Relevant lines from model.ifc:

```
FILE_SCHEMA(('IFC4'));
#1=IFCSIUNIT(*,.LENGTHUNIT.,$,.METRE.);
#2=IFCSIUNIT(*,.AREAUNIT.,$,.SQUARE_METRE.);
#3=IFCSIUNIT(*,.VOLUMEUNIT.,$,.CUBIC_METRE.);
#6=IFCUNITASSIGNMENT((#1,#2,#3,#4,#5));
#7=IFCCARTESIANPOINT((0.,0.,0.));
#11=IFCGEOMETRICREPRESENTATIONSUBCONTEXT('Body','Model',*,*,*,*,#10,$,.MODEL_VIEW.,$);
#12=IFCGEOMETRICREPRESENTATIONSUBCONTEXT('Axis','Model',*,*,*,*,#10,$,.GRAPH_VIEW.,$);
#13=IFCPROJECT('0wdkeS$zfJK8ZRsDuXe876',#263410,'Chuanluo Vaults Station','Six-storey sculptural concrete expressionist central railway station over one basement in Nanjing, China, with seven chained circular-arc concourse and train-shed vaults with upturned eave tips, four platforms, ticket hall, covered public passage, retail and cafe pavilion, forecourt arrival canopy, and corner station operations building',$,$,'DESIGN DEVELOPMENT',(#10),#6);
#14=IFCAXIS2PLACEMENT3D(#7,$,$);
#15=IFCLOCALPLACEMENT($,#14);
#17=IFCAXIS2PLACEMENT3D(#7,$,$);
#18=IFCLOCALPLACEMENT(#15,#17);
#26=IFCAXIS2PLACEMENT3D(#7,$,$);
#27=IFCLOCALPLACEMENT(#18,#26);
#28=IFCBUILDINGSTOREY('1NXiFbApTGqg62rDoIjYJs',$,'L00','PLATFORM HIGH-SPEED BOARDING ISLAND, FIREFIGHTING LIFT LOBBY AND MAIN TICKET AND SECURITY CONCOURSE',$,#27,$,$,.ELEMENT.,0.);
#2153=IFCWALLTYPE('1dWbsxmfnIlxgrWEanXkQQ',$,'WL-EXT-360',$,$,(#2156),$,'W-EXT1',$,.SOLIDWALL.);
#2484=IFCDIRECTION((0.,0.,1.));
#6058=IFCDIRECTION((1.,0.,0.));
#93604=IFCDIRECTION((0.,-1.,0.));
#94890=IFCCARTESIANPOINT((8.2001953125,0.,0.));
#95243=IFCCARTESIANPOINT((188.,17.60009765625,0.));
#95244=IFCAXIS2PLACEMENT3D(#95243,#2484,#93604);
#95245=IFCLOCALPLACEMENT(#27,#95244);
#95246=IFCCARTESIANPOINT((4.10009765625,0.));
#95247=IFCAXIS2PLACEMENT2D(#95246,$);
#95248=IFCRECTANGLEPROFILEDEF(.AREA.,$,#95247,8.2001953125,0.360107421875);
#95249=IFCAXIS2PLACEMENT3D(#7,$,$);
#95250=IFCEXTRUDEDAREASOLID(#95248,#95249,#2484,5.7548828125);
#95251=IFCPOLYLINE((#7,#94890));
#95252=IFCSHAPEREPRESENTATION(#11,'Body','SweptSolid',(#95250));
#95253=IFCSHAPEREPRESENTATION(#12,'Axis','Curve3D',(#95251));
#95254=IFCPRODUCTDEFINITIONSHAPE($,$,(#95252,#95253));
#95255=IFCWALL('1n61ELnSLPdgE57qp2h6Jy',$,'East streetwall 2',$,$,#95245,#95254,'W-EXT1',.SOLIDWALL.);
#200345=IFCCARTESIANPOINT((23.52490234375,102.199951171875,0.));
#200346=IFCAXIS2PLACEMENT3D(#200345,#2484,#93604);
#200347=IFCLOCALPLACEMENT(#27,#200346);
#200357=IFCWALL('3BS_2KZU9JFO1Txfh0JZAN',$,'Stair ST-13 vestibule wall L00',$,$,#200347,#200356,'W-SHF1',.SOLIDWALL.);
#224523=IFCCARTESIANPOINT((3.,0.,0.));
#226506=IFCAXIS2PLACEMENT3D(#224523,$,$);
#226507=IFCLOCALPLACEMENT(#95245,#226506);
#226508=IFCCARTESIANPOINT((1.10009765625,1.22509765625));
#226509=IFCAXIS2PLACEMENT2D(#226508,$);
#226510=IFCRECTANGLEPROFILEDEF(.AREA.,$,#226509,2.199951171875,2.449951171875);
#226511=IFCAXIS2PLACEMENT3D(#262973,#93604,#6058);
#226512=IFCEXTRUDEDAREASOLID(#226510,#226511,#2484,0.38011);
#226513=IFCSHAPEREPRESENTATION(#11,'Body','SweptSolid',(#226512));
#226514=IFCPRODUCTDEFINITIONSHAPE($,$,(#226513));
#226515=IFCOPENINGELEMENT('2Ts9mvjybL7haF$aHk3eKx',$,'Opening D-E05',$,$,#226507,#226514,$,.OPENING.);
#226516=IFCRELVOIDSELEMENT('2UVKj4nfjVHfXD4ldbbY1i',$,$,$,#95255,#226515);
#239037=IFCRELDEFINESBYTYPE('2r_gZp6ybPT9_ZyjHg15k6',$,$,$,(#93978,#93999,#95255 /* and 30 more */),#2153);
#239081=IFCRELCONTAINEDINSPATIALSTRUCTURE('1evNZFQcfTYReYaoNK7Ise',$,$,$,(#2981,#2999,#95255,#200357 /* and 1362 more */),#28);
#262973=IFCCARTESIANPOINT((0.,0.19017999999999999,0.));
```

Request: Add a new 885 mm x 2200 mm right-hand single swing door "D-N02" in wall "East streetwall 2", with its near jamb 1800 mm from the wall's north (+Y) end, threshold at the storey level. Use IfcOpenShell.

```python
import numpy as np
import ifcopenshell
import ifcopenshell.api.feature
import ifcopenshell.api.geometry
import ifcopenshell.api.root
import ifcopenshell.api.spatial
import ifcopenshell.geom
import ifcopenshell.util.element
import ifcopenshell.util.placement
import ifcopenshell.util.representation
import ifcopenshell.util.shape
import ifcopenshell.util.unit

model = ifcopenshell.open("model.ifc")
unit_scale = ifcopenshell.util.unit.calculate_unit_scale(model)
settings = ifcopenshell.geom.settings()


def volume(element):
    """Net volume in cubic metres, openings subtracted."""
    shape = ifcopenshell.geom.create_shape(settings, element)
    return ifcopenshell.util.shape.get_volume(shape.geometry)


wall = model.by_guid("1n61ELnSLPdgE57qp2h6Jy")
storey = ifcopenshell.util.element.get_container(wall, ifc_class="IfcBuildingStorey")
context = ifcopenshell.util.representation.get_context(model, "Model", "Body", "MODEL_VIEW")
before = volume(wall)

width, height, from_end, sill = 0.885, 2.2, 1.8, 0.0  # metres

# The wall runs along its own X axis, and the end named is its -X end.
wall_shape = ifcopenshell.geom.create_shape(settings, wall)
x, y, z = ifcopenshell.util.shape.get_vertices(wall_shape.geometry).T
start = x.min() + from_end
face, thickness = float(y.min()), float(y.max() - y.min())
wall_matrix = ifcopenshell.util.placement.get_local_placement(wall.ObjectPlacement)
level = ifcopenshell.util.placement.get_local_placement(storey.ObjectPlacement)[2, 3]


def in_wall(x, y):
    """Placement at x, y metres in the wall's axes, at sill height."""
    matrix = wall_matrix.copy()
    matrix[:, 3] = wall_matrix @ np.array([x / unit_scale, y / unit_scale, 0.0, 1.0])
    matrix[2, 3] = level + sill / unit_scale
    return matrix


# Opening: a box that overshoots both wall faces by 50 mm.
opening = ifcopenshell.api.root.create_entity(model, ifc_class="IfcOpeningElement", predefined_type="OPENING")
box = ifcopenshell.api.geometry.add_wall_representation(
    model, context=context, length=width, height=height, thickness=thickness + 0.1
)
ifcopenshell.api.geometry.assign_representation(model, product=opening, representation=box)
ifcopenshell.api.geometry.edit_object_placement(model, product=opening, matrix=in_wall(start, face - 0.05), is_si=False)
ifcopenshell.api.feature.add_feature(model, feature=opening, element=wall)

door = ifcopenshell.api.root.create_entity(model, ifc_class="IfcDoor", name="D-N02", predefined_type="DOOR")
door.OverallWidth, door.OverallHeight = width / unit_scale, height / unit_scale
door.OperationType = "SINGLE_SWING_RIGHT"
body = ifcopenshell.api.geometry.add_door_representation(
    model,
    context=context,
    overall_width=door.OverallWidth,
    overall_height=door.OverallHeight,
    operation_type="SINGLE_SWING_RIGHT",
    lining_properties={"LiningDepth": thickness / unit_scale, "ThresholdDepth": thickness / unit_scale},
)
ifcopenshell.api.geometry.assign_representation(model, product=door, representation=body)
ifcopenshell.api.spatial.assign_container(model, products=[door], relating_structure=storey)
ifcopenshell.api.feature.add_filling(model, opening=opening, element=door)

# The lining spans the wall, so the door starts at the wall face.
ifcopenshell.api.geometry.edit_object_placement(model, product=door, matrix=in_wall(start, face), is_si=False)

after = volume(wall)

print(f"wall volume {before:.3f} -> {after:.3f} m3")

model.write("model_updated.ifc")
```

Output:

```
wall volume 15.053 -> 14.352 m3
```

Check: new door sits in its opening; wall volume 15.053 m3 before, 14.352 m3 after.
